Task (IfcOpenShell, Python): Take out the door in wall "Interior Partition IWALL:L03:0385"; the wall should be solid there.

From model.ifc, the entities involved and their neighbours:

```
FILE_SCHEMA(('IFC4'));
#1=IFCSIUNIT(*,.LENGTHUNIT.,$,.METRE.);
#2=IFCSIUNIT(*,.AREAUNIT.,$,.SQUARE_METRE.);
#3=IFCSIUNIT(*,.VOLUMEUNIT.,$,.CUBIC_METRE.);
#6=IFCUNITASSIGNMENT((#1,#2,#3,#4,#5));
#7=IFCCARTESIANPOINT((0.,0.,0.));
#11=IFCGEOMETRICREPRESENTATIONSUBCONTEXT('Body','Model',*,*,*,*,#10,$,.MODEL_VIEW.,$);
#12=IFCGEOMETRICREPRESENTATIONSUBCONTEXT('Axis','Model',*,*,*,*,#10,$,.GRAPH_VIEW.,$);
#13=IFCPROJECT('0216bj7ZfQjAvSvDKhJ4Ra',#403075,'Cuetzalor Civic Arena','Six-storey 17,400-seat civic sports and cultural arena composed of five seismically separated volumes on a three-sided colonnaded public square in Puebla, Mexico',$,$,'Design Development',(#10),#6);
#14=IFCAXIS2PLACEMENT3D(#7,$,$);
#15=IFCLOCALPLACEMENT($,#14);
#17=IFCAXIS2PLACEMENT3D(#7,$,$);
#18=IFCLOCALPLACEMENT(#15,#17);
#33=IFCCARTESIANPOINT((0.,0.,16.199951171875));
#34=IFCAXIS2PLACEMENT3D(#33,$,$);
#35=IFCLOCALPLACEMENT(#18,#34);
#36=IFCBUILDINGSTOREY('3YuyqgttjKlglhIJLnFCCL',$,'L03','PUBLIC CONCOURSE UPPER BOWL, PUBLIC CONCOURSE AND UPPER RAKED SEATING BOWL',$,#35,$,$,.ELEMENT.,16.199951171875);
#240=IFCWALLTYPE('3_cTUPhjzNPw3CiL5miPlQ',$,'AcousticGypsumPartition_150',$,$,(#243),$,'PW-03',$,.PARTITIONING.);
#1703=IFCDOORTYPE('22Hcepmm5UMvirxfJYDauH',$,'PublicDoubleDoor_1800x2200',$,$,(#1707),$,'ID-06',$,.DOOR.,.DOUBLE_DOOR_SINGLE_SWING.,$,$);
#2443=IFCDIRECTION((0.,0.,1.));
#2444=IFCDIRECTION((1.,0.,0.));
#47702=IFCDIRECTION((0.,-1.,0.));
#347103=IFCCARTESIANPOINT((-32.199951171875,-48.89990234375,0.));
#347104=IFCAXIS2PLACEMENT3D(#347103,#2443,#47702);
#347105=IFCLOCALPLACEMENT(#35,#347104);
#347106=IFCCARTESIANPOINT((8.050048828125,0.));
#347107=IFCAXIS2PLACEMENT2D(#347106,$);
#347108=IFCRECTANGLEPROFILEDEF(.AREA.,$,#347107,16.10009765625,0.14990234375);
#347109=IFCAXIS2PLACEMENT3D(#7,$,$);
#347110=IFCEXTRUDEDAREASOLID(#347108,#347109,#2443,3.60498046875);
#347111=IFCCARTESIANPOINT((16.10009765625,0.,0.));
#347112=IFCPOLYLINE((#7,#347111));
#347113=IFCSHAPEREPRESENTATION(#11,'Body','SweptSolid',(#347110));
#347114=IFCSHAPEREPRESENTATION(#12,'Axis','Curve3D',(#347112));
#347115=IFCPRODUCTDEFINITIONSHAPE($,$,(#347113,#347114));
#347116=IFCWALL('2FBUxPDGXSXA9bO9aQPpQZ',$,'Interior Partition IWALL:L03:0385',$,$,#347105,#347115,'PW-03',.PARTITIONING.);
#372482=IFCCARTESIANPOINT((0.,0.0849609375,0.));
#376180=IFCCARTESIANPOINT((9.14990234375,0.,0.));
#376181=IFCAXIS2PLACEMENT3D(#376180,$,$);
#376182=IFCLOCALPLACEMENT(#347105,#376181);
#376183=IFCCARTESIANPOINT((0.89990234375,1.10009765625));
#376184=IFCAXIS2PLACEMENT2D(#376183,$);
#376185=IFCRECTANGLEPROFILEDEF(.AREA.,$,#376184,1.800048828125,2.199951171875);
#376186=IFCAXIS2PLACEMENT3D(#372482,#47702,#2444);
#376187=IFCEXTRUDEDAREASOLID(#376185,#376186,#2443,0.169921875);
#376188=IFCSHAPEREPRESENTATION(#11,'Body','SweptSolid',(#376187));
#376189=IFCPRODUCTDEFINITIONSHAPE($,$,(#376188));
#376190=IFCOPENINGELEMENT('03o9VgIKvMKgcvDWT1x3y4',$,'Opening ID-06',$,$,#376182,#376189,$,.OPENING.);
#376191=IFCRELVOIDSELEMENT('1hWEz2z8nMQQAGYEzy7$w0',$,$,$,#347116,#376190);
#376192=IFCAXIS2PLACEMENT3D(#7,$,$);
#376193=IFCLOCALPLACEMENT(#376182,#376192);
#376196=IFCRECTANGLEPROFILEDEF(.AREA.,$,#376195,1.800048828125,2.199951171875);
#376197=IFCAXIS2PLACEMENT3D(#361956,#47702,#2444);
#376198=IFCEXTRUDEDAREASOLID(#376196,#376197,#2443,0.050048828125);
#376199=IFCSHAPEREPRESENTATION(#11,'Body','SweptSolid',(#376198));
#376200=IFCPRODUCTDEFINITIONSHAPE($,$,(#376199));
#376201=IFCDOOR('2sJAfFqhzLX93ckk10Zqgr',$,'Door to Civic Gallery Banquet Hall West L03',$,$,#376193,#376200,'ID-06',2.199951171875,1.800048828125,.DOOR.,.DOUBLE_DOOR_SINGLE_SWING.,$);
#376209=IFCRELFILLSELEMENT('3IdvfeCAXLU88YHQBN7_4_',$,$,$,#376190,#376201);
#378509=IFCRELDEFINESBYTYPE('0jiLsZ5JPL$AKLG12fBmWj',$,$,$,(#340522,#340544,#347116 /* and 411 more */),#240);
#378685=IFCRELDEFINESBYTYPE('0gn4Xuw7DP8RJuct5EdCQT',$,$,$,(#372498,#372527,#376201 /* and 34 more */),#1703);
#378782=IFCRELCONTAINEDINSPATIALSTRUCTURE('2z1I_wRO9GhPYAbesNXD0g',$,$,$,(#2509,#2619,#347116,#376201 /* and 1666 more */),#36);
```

```python
import ifcopenshell
import ifcopenshell.api.feature
import ifcopenshell.api.root
import ifcopenshell.geom
import ifcopenshell.util.shape

model = ifcopenshell.open("model.ifc")
settings = ifcopenshell.geom.settings()


def volume(element):
    """Net volume in cubic metres, openings subtracted."""
    shape = ifcopenshell.geom.create_shape(settings, element)
    return ifcopenshell.util.shape.get_volume(shape.geometry)


door = model.by_id(376201)
opening = door.FillsVoids[0].RelatingOpeningElement
wall = opening.VoidsElements[0].RelatingBuildingElement
before = volume(wall)

ifcopenshell.api.root.remove_product(model, product=door)
ifcopenshell.api.feature.remove_feature(model, feature=opening)

after = volume(wall)

print(f"wall volume {before:.3f} -> {after:.3f} m3")

model.write("model_v2.ifc")
```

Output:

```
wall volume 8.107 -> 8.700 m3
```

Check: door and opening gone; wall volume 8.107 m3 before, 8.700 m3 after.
